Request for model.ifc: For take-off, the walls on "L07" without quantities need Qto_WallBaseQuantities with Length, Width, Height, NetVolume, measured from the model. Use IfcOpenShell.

First a look at what the model holds.

```python
import ifcopenshell
import ifcopenshell.util.element
import ifcopenshell.util.unit

model = ifcopenshell.open("model.ifc")
print(model.schema)
for unit_type in ("LENGTHUNIT", "AREAUNIT", "VOLUMEUNIT"):
    print(unit_type, ifcopenshell.util.unit.calculate_unit_scale(model, unit_type))
storey = next(s for s in model.by_type("IfcBuildingStorey") if s.Name == "L07")
walls = [e for e in ifcopenshell.util.element.get_decomposition(storey) if e.is_a("IfcWall")]
for e in sorted(walls, key=lambda e: e.id()):
    print(e.id(), e.is_a(), e.Name, list(ifcopenshell.util.element.get_psets(e, qtos_only=True)), sep=" | ")
```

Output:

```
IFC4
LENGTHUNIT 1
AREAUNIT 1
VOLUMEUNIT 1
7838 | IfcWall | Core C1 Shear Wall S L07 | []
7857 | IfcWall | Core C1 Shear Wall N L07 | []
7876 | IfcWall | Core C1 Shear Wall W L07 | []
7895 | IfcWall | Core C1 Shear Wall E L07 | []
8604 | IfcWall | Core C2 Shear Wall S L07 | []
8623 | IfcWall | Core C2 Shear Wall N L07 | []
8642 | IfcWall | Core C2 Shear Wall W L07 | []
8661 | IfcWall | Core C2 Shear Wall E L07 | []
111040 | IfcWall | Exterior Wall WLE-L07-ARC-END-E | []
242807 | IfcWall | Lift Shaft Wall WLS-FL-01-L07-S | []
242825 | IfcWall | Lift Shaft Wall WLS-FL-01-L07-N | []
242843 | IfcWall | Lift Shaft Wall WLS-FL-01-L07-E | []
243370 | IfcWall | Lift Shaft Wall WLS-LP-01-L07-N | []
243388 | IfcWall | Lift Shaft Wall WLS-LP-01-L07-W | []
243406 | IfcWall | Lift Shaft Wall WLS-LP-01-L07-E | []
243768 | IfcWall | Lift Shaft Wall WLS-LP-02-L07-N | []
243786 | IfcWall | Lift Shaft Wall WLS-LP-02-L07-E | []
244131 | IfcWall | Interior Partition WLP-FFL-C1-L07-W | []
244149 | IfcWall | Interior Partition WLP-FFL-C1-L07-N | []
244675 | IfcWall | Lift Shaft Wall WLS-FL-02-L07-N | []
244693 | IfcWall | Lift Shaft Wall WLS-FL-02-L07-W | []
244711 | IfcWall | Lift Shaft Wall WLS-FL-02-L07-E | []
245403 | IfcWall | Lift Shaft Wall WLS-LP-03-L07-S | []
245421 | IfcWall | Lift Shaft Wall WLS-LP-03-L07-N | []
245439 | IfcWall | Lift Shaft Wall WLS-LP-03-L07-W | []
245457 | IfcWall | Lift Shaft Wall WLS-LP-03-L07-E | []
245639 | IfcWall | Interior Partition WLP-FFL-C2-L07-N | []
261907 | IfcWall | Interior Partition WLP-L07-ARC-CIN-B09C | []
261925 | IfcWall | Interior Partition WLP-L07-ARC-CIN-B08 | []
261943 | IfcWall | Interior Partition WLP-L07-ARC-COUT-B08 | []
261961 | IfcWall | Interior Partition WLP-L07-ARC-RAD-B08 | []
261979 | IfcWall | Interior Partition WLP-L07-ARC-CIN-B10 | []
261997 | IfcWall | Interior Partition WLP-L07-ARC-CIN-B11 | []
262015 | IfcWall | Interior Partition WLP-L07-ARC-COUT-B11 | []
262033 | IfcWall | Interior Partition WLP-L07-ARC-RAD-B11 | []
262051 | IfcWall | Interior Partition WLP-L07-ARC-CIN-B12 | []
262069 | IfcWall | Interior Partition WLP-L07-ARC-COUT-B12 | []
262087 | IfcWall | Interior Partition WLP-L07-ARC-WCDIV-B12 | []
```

```python
import ifcopenshell
import ifcopenshell.api.pset
import ifcopenshell.geom
import ifcopenshell.util.element
import ifcopenshell.util.shape
import ifcopenshell.util.unit

model = ifcopenshell.open("model.ifc")
unit_scale = ifcopenshell.util.unit.calculate_unit_scale(model)
volume_scale = ifcopenshell.util.unit.calculate_unit_scale(model, "VOLUMEUNIT")
settings = ifcopenshell.geom.settings()

storey = next(s for s in model.by_type("IfcBuildingStorey") if s.Name == "L07")
walls = [e for e in ifcopenshell.util.element.get_decomposition(storey) if e.is_a("IfcWall")]

for e in sorted(walls, key=lambda e: e.id()):
    if ifcopenshell.util.element.get_psets(e, qtos_only=True, should_inherit=False):
        continue
    # Geometry comes back in metres, in the element's own axes.
    shape = ifcopenshell.geom.create_shape(settings, e)
    values = {
        "Length": ifcopenshell.util.shape.get_x(shape.geometry) / unit_scale,
        "Width": ifcopenshell.util.shape.get_y(shape.geometry) / unit_scale,
        "Height": ifcopenshell.util.shape.get_z(shape.geometry) / unit_scale,
        "NetVolume": ifcopenshell.util.shape.get_volume(shape.geometry) / volume_scale,
    }
    qto = ifcopenshell.api.pset.add_qto(model, product=e, name="Qto_WallBaseQuantities")
    ifcopenshell.api.pset.edit_qto(model, qto=qto, properties=values)
    print(e.id(), {k: round(v, 3) for k, v in values.items()})

model.write("model_edited.ifc")
```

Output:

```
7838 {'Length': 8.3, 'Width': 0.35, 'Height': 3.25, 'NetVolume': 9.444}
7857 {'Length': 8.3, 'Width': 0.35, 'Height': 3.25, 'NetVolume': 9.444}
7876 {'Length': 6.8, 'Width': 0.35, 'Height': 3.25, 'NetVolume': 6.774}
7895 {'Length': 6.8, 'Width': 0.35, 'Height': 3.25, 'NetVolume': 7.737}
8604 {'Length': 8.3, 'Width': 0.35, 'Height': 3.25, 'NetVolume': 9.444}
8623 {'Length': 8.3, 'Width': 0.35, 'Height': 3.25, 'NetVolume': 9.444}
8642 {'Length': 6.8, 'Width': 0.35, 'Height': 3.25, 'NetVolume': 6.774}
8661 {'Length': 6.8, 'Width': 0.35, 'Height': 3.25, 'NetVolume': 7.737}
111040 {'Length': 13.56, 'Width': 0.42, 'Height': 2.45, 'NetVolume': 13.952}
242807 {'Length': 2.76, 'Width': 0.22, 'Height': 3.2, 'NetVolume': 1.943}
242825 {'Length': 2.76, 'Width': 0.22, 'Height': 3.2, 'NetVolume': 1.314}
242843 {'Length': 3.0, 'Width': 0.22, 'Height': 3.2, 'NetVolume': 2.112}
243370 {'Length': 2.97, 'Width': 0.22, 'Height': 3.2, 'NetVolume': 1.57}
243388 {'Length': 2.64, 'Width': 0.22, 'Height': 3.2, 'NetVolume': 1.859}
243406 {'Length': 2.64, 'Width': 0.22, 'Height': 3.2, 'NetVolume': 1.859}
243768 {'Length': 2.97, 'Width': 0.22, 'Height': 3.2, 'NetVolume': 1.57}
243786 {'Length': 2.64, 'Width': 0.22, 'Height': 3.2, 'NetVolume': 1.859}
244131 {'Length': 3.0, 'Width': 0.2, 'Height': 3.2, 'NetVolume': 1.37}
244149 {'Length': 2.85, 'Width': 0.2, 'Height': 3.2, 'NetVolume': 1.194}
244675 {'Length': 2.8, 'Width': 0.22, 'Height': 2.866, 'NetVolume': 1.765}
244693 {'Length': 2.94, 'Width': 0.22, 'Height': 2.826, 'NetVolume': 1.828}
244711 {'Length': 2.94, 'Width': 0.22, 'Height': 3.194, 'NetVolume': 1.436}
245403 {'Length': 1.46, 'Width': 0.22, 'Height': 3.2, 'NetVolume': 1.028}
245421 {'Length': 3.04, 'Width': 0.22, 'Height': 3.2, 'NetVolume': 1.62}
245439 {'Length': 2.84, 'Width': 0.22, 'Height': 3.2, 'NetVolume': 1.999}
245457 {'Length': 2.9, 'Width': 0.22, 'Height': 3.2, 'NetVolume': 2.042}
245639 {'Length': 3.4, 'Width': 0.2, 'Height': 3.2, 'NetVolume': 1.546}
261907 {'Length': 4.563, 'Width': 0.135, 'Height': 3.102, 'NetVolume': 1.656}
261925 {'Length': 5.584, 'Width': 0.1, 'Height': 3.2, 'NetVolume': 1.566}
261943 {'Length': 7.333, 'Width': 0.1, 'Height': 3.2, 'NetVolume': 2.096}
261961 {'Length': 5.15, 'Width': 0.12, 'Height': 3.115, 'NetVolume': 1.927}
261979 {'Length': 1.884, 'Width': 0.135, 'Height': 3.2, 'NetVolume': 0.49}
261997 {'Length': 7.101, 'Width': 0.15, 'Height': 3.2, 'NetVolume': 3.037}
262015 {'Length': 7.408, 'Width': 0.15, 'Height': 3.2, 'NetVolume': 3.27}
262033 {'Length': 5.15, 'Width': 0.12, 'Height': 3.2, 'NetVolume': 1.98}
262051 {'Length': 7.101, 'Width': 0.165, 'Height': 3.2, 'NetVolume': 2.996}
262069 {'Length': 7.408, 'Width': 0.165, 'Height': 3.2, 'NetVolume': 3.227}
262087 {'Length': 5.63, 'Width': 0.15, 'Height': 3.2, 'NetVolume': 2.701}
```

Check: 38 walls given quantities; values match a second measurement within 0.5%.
